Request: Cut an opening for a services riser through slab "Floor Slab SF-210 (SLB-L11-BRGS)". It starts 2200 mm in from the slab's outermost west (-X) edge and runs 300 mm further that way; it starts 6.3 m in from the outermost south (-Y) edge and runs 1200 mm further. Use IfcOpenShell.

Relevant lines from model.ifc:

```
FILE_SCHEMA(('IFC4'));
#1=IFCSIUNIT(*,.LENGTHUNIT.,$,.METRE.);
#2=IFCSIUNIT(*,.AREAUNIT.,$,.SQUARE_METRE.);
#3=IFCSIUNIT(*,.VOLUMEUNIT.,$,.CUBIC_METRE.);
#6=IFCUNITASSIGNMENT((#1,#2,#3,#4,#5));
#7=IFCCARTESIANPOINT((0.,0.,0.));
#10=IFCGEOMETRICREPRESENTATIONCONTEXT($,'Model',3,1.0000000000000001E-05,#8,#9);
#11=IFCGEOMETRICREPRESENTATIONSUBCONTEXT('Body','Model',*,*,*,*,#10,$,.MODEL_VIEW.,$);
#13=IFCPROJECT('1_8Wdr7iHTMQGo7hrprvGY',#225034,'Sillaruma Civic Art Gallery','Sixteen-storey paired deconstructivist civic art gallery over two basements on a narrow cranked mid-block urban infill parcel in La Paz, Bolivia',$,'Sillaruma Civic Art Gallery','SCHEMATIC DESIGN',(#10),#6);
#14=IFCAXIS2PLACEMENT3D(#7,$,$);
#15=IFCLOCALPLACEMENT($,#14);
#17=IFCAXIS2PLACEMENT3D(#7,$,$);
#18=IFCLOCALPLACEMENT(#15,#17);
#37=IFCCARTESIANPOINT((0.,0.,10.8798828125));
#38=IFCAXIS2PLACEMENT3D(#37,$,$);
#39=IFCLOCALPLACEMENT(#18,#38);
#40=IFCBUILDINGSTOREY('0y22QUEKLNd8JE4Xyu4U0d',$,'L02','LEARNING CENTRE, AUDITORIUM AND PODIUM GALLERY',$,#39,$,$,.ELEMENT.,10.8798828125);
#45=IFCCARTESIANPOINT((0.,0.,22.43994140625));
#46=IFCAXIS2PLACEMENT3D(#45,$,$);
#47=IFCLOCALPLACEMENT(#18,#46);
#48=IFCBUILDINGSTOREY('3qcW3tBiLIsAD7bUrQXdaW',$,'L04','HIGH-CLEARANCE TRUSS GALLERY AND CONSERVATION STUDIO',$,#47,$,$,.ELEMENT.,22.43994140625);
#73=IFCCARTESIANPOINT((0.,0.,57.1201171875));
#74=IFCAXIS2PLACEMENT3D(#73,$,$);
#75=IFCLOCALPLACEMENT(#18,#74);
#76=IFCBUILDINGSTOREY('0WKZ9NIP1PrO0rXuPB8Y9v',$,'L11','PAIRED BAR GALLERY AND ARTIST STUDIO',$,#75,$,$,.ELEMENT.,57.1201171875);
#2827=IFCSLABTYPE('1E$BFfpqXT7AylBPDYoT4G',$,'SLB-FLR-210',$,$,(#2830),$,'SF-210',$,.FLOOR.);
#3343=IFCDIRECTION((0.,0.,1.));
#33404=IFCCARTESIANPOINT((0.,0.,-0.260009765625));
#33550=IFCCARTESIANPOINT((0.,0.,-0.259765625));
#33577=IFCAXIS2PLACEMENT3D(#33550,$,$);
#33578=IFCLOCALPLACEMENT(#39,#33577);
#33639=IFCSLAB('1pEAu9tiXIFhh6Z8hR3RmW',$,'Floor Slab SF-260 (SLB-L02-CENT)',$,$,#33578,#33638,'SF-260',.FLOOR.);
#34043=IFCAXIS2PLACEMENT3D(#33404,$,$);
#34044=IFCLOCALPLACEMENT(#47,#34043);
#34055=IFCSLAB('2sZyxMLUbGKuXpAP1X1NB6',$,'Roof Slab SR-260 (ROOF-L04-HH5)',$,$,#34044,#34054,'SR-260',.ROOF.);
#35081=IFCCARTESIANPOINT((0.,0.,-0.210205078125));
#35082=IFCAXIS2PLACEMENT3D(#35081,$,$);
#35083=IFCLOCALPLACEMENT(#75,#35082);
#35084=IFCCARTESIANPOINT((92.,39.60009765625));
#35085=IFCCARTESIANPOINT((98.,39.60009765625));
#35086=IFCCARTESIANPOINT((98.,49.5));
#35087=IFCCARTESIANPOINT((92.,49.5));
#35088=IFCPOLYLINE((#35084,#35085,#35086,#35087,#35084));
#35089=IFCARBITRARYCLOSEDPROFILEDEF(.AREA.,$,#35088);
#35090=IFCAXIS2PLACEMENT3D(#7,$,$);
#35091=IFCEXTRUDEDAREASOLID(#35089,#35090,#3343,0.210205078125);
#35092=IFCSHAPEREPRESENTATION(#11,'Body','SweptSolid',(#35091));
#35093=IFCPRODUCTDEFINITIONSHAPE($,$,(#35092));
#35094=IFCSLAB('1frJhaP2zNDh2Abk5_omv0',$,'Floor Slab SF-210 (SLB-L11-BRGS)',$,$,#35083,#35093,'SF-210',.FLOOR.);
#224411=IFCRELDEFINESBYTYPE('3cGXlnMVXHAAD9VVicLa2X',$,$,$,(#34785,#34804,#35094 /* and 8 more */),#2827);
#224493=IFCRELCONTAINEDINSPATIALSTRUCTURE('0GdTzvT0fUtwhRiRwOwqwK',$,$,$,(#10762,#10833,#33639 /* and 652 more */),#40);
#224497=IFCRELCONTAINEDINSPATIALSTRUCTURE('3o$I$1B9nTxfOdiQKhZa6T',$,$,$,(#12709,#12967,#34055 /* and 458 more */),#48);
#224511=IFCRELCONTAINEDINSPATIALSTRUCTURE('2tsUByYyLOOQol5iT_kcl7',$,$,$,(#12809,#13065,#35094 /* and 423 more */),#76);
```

```python
import numpy as np
import ifcopenshell
import ifcopenshell.api.feature
import ifcopenshell.api.geometry
import ifcopenshell.api.root
import ifcopenshell.geom
import ifcopenshell.util.placement
import ifcopenshell.util.representation
import ifcopenshell.util.shape
import ifcopenshell.util.unit

model = ifcopenshell.open("model.ifc")
unit_scale = ifcopenshell.util.unit.calculate_unit_scale(model)
settings = ifcopenshell.geom.settings()


def volume(element):
    """Net volume in cubic metres, openings subtracted."""
    shape = ifcopenshell.geom.create_shape(settings, element)
    return ifcopenshell.util.shape.get_volume(shape.geometry)


slab = model.by_guid("1frJhaP2zNDh2Abk5_omv0")
before = volume(slab)

# Extent in the slab's own axes, in metres. The edges named are its -X and -Y sides.
slab_shape = ifcopenshell.geom.create_shape(settings, slab)
vertices = ifcopenshell.util.shape.get_vertices(slab_shape.geometry)
x_min, y_min, bottom = vertices.min(axis=0)
top = vertices[:, 2].max()

opening = ifcopenshell.api.root.create_entity(model, ifc_class="IfcOpeningElement", name="Services riser opening", predefined_type="OPENING")
context = ifcopenshell.util.representation.get_context(model, "Model", "Body", "MODEL_VIEW")
width, depth = 0.3, 1.2
outline = [(0.0, 0.0), (width, 0.0), (width, depth), (0.0, depth), (0.0, 0.0)]
# Overshoot both faces by 50 mm so the cut is clean.
shape = ifcopenshell.api.geometry.add_slab_representation(
    model, context=context, depth=top - bottom + 0.1, polyline=outline
)
ifcopenshell.api.geometry.assign_representation(model, product=opening, representation=shape)

matrix = ifcopenshell.util.placement.get_local_placement(slab.ObjectPlacement)
matrix[:, 3] = matrix @ np.append(np.array([x_min + 2.2, y_min + 6.3, bottom - 0.05]) / unit_scale, 1.0)
ifcopenshell.api.geometry.edit_object_placement(model, product=opening, matrix=matrix, is_si=False)
ifcopenshell.api.feature.add_feature(model, feature=opening, element=slab)

after = volume(slab)

print(f"slab volume {before:.3f} -> {after:.3f} m3")

model.write("model_v2.ifc")
```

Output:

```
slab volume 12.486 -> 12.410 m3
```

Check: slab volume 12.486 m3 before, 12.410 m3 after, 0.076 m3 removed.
